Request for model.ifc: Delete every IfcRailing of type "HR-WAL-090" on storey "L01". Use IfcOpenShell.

First a look at what the model holds.

```python
import ifcopenshell
import ifcopenshell.util.element

model = ifcopenshell.open("model.ifc")
print(model.schema)
storey = next(s for s in model.by_type("IfcBuildingStorey") if s.Name == "L01")
railings = [e for e in ifcopenshell.util.element.get_decomposition(storey) if e.is_a("IfcRailing")]
seen = {}
for e in railings:
    element_type = ifcopenshell.util.element.get_type(e)
    name = element_type.Name if element_type not in (None, e) else None
    seen[name] = seen.get(name, 0) + 1
for name, count in sorted(seen.items(), key=str):
    print(count, "x", name)
```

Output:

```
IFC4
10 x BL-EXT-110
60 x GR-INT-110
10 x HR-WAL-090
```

```python
import ifcopenshell
import ifcopenshell.api.root
import ifcopenshell.util.element

model = ifcopenshell.open("model.ifc")

storey = next(s for s in model.by_type("IfcBuildingStorey") if s.Name == "L01")
railings = [e for e in ifcopenshell.util.element.get_decomposition(storey) if e.is_a("IfcRailing")]
targets = [e for e in railings if (t := ifcopenshell.util.element.get_type(e)) not in (None, e) and t.Name == "HR-WAL-090"]

for e in targets:
    ifcopenshell.api.root.remove_product(model, product=e)
print(len(targets), "removed")

model.write("model_v2.ifc")
```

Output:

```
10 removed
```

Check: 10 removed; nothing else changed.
